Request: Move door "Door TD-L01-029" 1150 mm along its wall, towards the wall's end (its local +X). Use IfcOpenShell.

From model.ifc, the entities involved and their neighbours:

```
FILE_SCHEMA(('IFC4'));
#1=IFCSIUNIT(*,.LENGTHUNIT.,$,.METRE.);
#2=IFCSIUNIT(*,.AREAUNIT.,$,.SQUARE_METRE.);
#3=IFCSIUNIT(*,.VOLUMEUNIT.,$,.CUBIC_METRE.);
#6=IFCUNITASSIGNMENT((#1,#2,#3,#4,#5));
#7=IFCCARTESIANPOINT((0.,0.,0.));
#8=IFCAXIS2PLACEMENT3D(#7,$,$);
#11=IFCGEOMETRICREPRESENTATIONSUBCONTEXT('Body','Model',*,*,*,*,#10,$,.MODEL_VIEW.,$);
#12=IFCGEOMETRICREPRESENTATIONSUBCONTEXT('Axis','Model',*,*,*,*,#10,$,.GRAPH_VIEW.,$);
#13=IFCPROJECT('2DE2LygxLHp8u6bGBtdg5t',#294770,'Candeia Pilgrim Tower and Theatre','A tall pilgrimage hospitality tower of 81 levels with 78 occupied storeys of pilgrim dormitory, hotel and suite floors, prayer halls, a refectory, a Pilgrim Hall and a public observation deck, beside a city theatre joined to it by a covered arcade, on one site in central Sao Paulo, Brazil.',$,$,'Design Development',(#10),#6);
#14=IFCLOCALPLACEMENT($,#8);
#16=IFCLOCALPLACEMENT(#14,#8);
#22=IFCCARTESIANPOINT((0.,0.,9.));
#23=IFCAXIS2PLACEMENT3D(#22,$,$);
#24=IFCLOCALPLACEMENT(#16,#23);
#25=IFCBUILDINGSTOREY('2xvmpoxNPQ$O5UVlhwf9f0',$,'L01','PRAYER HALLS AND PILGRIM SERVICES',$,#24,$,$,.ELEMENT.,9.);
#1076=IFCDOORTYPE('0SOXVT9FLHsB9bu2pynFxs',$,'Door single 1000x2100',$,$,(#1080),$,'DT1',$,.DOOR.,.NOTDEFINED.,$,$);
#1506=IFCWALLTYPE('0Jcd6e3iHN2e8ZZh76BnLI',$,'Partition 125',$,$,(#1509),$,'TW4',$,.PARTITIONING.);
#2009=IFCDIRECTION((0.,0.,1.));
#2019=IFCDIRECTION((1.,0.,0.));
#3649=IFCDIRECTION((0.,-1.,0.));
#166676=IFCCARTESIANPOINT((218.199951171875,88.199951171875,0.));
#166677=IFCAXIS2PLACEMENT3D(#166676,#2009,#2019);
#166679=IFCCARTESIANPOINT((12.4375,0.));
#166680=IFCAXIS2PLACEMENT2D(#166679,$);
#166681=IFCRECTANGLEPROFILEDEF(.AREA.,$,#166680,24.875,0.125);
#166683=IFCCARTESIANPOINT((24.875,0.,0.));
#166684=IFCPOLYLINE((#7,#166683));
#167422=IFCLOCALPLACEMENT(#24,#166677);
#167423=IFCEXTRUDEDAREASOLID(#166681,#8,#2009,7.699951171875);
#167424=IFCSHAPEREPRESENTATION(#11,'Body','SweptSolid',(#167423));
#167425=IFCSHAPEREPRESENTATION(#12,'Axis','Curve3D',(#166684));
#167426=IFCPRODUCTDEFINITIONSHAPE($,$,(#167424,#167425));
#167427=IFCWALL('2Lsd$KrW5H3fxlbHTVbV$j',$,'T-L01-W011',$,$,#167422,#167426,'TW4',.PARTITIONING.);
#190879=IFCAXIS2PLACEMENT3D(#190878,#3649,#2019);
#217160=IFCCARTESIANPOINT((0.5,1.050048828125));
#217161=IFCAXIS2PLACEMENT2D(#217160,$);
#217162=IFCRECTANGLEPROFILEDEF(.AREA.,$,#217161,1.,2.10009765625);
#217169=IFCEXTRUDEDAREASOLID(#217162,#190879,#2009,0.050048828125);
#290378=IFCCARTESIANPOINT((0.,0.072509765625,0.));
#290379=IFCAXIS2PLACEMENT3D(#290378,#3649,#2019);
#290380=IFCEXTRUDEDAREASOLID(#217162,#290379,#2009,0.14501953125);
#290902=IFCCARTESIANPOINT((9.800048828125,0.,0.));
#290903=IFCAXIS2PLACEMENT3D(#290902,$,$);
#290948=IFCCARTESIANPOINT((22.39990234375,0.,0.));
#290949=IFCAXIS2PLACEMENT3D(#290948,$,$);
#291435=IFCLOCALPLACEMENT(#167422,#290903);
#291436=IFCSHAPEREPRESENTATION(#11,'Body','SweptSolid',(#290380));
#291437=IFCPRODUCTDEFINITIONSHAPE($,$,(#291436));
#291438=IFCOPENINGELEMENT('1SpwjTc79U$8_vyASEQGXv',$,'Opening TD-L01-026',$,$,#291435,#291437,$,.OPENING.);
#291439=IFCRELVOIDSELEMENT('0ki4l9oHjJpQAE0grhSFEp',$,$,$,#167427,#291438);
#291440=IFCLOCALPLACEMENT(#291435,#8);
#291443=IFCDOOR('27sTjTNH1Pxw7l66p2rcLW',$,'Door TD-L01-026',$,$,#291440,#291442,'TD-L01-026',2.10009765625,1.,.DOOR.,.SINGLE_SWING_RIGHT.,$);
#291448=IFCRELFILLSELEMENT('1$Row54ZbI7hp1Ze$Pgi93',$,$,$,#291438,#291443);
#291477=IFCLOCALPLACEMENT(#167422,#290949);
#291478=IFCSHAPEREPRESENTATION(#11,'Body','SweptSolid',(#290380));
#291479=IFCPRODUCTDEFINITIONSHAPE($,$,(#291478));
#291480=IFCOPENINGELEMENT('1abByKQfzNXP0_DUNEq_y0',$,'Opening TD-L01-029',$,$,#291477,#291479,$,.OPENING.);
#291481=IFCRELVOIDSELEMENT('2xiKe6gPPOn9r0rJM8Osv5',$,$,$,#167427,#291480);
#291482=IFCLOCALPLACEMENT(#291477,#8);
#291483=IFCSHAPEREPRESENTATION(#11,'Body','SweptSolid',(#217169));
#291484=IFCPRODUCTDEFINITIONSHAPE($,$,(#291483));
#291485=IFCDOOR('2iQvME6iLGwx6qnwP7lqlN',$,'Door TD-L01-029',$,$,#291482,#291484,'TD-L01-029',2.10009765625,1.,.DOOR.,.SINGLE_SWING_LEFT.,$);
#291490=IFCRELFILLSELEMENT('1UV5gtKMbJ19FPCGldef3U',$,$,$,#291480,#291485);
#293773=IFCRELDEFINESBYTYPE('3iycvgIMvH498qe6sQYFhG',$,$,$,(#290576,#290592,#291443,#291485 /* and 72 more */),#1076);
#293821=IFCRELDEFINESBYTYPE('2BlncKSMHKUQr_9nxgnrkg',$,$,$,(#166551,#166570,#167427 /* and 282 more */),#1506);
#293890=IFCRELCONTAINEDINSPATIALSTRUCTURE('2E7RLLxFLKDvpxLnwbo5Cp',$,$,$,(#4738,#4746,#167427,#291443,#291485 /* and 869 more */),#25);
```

```python
import ifcopenshell
import ifcopenshell.api.geometry
import ifcopenshell.util.placement
import ifcopenshell.util.unit

model = ifcopenshell.open("model.ifc")
unit_scale = ifcopenshell.util.unit.calculate_unit_scale(model)

door = model.by_id(291485)
opening = door.FillsVoids[0].RelatingOpeningElement
wall = opening.VoidsElements[0].RelatingBuildingElement

wall_matrix = ifcopenshell.util.placement.get_local_placement(wall.ObjectPlacement)
shift = wall_matrix[:3, 0] * 1.15 / unit_scale
before = ifcopenshell.util.placement.get_local_placement(door.ObjectPlacement)[:3, 3].copy()

# The door is placed relative to its opening, so it follows when the opening moves.
matrix = ifcopenshell.util.placement.get_local_placement(opening.ObjectPlacement)
matrix[:3, 3] += shift
ifcopenshell.api.geometry.edit_object_placement(
    model, product=opening, matrix=matrix, is_si=False, should_transform_children=True
)

after = ifcopenshell.util.placement.get_local_placement(door.ObjectPlacement)[:3, 3]
print("door moved by", (after - before).round(3) + 0.0)

model.write("model_updated.ifc")
```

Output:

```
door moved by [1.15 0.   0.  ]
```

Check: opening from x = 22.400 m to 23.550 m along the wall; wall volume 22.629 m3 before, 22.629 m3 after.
